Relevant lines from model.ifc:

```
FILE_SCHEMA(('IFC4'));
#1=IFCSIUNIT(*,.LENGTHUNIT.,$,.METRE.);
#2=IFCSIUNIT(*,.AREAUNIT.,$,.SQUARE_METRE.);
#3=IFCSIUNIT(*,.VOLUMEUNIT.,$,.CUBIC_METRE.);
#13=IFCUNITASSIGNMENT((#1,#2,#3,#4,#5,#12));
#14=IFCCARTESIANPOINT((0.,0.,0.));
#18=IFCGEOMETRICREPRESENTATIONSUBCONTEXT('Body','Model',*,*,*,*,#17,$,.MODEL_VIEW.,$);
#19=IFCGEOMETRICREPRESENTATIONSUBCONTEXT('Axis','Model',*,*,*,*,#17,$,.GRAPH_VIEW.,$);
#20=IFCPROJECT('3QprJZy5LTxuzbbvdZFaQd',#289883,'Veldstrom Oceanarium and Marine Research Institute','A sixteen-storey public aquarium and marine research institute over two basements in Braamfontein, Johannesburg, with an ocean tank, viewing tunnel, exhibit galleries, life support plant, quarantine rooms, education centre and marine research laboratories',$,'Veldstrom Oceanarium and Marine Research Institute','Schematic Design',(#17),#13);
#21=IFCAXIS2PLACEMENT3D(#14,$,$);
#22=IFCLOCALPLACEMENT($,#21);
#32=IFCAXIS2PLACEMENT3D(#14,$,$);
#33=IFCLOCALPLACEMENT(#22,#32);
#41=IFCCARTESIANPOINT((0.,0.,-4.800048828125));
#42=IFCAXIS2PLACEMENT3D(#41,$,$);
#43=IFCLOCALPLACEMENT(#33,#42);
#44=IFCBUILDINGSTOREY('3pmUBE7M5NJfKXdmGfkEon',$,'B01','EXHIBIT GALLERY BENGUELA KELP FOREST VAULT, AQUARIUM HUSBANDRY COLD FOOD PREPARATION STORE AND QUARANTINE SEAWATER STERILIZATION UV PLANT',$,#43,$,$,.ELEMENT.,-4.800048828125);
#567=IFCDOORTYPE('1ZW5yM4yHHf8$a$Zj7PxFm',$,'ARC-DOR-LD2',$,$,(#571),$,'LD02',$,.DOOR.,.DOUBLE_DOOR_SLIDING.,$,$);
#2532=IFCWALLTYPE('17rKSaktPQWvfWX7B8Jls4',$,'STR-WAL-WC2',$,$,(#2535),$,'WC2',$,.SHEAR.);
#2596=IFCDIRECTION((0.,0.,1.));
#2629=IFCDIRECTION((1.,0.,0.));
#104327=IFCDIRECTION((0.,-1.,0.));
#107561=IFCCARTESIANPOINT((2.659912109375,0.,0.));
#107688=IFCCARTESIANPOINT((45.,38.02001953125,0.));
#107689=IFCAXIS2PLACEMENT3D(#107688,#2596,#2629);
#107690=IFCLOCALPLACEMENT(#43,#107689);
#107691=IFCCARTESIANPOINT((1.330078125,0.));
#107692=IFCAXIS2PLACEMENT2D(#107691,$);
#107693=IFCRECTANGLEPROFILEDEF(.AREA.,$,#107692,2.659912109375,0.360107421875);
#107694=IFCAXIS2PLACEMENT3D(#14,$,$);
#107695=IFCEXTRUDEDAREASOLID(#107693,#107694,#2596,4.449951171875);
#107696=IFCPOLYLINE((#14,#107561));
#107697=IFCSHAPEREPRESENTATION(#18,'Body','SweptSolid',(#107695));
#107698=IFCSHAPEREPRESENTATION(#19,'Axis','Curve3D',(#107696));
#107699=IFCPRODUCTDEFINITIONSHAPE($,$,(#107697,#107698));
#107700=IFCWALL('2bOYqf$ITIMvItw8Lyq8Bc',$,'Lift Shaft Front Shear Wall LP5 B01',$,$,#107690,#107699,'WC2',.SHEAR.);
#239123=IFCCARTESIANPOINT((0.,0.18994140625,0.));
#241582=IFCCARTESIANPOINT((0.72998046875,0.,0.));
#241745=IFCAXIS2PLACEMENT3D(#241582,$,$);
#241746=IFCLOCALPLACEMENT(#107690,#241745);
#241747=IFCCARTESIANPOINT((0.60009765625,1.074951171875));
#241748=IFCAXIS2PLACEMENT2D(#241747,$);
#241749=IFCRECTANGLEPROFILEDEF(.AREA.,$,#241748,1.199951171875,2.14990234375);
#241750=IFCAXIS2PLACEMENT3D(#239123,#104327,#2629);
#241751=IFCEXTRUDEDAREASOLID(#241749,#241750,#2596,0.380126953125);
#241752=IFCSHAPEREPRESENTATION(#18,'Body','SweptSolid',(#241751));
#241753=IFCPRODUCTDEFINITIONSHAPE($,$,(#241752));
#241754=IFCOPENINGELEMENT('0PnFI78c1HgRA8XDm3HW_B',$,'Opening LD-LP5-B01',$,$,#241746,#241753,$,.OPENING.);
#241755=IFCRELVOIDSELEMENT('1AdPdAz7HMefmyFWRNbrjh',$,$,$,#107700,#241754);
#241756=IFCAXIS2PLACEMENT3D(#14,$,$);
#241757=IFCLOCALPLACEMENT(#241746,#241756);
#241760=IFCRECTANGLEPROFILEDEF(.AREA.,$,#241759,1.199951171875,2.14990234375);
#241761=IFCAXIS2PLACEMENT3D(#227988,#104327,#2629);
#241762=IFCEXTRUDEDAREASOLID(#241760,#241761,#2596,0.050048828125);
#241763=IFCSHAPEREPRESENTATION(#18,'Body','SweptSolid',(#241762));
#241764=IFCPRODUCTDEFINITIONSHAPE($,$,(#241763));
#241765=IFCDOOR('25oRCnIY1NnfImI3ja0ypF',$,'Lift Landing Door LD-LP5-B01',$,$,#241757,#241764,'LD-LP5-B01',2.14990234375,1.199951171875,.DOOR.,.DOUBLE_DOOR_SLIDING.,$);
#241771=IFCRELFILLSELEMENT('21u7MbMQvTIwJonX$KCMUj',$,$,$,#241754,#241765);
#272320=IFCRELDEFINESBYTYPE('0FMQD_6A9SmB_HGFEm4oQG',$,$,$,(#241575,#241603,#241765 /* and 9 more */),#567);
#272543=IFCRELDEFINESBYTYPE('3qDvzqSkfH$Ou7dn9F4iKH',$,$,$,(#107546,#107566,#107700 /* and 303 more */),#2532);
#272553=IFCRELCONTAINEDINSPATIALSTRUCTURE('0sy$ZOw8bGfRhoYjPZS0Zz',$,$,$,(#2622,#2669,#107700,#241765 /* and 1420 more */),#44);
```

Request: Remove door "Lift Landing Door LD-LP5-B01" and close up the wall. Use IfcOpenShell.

```python
import ifcopenshell
import ifcopenshell.api.feature
import ifcopenshell.api.root
import ifcopenshell.geom
import ifcopenshell.util.shape

model = ifcopenshell.open("model.ifc")
settings = ifcopenshell.geom.settings()


def volume(element):
    """Net volume in cubic metres, openings subtracted."""
    shape = ifcopenshell.geom.create_shape(settings, element)
    return ifcopenshell.util.shape.get_volume(shape.geometry)


door = model.by_id(241765)
opening = door.FillsVoids[0].RelatingOpeningElement
wall = opening.VoidsElements[0].RelatingBuildingElement
before = volume(wall)

ifcopenshell.api.root.remove_product(model, product=door)
ifcopenshell.api.feature.remove_feature(model, feature=opening)

after = volume(wall)

print(f"wall volume {before:.3f} -> {after:.3f} m3")

model.write("model_rev.ifc")
```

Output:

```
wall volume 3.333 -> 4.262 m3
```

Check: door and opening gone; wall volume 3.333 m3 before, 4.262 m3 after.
